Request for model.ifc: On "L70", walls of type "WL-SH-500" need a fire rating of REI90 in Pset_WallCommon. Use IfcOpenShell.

First a look at what the model holds.

```python
import ifcopenshell
import ifcopenshell.util.element

model = ifcopenshell.open("model.ifc")
print(model.schema)
storey = next(s for s in model.by_type("IfcBuildingStorey") if s.Name == "L70")
walls = [e for e in ifcopenshell.util.element.get_decomposition(storey) if e.is_a("IfcWall")]
seen = {}
for e in walls:
    element_type = ifcopenshell.util.element.get_type(e)
    key = (element_type.Name if element_type != e and element_type else None, ifcopenshell.util.element.get_pset(e, "Pset_WallCommon", "FireRating"))
    seen[key] = seen.get(key, 0) + 1
for (name, value), count in sorted(seen.items(), key=str):
    print(count, "x", name, "|", value)
```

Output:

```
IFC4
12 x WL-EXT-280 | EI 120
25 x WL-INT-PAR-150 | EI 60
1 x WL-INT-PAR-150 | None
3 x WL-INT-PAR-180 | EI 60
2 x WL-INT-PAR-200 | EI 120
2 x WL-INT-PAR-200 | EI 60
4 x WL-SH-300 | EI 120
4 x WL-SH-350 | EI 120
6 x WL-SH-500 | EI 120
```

```python
import ifcopenshell
import ifcopenshell.api.pset
import ifcopenshell.util.element

model = ifcopenshell.open("model.ifc")

storey = next(s for s in model.by_type("IfcBuildingStorey") if s.Name == "L70")
walls = [e for e in ifcopenshell.util.element.get_decomposition(storey) if e.is_a("IfcWall")]

count = 0
for e in walls:
    element_type = ifcopenshell.util.element.get_type(e)
    if element_type in (None, e) or element_type.Name != "WL-SH-500":
        continue
    found = ifcopenshell.util.element.get_pset(e, "Pset_WallCommon", should_inherit=False)
    if found:
        pset = model.by_id(found["id"])
        if len(ifcopenshell.util.element.get_elements_by_pset(pset)) > 1:
            pset = ifcopenshell.api.pset.unshare_pset(model, products=[e], pset=pset)[0]
    else:
        pset = ifcopenshell.api.pset.add_pset(model, product=e, name="Pset_WallCommon")
    ifcopenshell.api.pset.edit_pset(model, pset=pset, properties={"FireRating": "REI90"})
    count += 1

print(count, "walls updated")

model.write("model-out.ifc")
```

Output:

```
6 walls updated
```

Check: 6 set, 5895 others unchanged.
